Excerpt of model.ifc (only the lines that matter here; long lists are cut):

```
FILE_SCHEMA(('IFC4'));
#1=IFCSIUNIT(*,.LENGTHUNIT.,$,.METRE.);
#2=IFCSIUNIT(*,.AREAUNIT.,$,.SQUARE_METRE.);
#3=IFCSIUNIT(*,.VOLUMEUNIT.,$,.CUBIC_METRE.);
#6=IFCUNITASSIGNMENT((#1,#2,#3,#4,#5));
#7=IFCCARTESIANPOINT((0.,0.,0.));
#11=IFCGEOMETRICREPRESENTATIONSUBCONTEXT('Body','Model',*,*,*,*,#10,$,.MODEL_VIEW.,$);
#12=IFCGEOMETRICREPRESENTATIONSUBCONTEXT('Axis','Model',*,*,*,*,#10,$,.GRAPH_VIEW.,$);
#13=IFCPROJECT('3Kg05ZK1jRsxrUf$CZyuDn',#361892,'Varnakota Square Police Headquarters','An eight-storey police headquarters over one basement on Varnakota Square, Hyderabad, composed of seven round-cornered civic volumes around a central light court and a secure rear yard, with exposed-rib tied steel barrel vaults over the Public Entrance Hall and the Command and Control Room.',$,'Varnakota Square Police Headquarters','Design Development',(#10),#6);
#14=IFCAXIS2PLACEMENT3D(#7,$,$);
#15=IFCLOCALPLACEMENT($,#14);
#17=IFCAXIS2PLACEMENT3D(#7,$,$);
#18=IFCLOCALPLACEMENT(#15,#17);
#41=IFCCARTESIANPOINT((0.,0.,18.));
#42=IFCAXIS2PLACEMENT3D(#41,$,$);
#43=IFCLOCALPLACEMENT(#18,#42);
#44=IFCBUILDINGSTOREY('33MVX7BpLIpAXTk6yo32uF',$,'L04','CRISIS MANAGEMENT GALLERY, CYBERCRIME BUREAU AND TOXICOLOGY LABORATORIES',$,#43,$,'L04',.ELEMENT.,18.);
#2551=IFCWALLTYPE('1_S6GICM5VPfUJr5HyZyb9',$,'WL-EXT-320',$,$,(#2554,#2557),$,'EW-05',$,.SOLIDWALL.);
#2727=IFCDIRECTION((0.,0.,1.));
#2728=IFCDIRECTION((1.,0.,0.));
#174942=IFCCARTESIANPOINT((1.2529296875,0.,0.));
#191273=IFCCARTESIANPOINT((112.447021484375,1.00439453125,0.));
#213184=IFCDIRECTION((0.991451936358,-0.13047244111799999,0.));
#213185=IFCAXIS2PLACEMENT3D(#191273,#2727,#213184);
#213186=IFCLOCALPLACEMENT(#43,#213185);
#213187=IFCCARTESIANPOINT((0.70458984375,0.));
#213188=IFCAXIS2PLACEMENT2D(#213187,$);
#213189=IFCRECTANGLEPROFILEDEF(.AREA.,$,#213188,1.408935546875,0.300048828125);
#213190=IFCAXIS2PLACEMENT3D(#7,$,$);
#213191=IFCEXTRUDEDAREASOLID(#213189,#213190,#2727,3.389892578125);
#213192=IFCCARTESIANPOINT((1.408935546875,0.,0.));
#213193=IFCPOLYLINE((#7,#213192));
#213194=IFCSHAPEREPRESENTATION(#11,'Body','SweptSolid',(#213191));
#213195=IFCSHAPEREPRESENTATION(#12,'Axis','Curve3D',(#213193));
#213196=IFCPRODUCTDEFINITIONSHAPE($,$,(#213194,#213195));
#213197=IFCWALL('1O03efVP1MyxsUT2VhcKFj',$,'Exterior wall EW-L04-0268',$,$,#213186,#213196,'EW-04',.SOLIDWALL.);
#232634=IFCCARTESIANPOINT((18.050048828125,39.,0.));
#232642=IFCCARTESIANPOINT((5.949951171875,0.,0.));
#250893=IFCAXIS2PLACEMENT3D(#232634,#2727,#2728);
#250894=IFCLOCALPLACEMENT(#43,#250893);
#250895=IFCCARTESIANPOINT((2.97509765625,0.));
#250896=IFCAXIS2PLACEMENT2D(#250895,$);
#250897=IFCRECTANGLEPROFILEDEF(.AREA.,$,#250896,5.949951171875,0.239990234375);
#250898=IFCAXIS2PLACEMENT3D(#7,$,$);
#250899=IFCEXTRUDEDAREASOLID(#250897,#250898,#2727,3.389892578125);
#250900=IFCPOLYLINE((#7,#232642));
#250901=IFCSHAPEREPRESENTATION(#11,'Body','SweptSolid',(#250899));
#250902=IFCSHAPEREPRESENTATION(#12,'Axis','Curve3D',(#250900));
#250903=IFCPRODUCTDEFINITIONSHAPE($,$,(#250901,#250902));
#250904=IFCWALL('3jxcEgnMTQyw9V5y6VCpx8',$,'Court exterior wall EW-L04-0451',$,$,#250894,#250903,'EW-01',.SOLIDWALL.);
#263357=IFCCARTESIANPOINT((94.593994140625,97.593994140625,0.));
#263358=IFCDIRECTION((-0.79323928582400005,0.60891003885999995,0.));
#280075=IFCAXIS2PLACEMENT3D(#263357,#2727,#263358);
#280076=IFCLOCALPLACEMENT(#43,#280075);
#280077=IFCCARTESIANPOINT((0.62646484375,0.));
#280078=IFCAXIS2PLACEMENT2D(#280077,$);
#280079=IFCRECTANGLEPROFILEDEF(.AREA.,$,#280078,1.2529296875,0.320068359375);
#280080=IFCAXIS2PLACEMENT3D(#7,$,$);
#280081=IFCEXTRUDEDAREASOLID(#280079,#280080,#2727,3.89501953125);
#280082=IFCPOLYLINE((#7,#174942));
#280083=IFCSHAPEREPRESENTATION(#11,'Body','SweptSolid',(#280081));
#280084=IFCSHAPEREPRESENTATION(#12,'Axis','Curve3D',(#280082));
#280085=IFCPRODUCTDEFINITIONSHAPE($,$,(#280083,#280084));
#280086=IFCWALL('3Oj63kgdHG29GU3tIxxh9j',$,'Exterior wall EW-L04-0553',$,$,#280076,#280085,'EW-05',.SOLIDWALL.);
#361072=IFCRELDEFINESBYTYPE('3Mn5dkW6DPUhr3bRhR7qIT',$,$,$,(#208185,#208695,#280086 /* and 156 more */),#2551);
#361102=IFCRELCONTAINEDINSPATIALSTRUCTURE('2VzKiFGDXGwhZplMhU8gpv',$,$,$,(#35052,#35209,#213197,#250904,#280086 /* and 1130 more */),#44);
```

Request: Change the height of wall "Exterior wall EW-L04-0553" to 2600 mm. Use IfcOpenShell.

```python
import ifcopenshell
import ifcopenshell.geom
import ifcopenshell.util.representation
import ifcopenshell.util.shape
import ifcopenshell.util.unit

model = ifcopenshell.open("model.ifc")
unit_scale = ifcopenshell.util.unit.calculate_unit_scale(model)
settings = ifcopenshell.geom.settings()


def volume(element):
    """Net volume in cubic metres, openings subtracted."""
    shape = ifcopenshell.geom.create_shape(settings, element)
    return ifcopenshell.util.shape.get_volume(shape.geometry)


wall = model.by_guid("3Oj63kgdHG29GU3tIxxh9j")
before = volume(wall)

body = ifcopenshell.util.representation.get_representation(wall, "Model", "Body")
solid = body.Items[0]
old_height = solid.Depth
solid.Depth = 2.6 / unit_scale
after = volume(wall)

print(f"height {old_height:g} -> {solid.Depth:g}, volume {before:.3f} -> {after:.3f} m3")

model.write("model_rev.ifc")
```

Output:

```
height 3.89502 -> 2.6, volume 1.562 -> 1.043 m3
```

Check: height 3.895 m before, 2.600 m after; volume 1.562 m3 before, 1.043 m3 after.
